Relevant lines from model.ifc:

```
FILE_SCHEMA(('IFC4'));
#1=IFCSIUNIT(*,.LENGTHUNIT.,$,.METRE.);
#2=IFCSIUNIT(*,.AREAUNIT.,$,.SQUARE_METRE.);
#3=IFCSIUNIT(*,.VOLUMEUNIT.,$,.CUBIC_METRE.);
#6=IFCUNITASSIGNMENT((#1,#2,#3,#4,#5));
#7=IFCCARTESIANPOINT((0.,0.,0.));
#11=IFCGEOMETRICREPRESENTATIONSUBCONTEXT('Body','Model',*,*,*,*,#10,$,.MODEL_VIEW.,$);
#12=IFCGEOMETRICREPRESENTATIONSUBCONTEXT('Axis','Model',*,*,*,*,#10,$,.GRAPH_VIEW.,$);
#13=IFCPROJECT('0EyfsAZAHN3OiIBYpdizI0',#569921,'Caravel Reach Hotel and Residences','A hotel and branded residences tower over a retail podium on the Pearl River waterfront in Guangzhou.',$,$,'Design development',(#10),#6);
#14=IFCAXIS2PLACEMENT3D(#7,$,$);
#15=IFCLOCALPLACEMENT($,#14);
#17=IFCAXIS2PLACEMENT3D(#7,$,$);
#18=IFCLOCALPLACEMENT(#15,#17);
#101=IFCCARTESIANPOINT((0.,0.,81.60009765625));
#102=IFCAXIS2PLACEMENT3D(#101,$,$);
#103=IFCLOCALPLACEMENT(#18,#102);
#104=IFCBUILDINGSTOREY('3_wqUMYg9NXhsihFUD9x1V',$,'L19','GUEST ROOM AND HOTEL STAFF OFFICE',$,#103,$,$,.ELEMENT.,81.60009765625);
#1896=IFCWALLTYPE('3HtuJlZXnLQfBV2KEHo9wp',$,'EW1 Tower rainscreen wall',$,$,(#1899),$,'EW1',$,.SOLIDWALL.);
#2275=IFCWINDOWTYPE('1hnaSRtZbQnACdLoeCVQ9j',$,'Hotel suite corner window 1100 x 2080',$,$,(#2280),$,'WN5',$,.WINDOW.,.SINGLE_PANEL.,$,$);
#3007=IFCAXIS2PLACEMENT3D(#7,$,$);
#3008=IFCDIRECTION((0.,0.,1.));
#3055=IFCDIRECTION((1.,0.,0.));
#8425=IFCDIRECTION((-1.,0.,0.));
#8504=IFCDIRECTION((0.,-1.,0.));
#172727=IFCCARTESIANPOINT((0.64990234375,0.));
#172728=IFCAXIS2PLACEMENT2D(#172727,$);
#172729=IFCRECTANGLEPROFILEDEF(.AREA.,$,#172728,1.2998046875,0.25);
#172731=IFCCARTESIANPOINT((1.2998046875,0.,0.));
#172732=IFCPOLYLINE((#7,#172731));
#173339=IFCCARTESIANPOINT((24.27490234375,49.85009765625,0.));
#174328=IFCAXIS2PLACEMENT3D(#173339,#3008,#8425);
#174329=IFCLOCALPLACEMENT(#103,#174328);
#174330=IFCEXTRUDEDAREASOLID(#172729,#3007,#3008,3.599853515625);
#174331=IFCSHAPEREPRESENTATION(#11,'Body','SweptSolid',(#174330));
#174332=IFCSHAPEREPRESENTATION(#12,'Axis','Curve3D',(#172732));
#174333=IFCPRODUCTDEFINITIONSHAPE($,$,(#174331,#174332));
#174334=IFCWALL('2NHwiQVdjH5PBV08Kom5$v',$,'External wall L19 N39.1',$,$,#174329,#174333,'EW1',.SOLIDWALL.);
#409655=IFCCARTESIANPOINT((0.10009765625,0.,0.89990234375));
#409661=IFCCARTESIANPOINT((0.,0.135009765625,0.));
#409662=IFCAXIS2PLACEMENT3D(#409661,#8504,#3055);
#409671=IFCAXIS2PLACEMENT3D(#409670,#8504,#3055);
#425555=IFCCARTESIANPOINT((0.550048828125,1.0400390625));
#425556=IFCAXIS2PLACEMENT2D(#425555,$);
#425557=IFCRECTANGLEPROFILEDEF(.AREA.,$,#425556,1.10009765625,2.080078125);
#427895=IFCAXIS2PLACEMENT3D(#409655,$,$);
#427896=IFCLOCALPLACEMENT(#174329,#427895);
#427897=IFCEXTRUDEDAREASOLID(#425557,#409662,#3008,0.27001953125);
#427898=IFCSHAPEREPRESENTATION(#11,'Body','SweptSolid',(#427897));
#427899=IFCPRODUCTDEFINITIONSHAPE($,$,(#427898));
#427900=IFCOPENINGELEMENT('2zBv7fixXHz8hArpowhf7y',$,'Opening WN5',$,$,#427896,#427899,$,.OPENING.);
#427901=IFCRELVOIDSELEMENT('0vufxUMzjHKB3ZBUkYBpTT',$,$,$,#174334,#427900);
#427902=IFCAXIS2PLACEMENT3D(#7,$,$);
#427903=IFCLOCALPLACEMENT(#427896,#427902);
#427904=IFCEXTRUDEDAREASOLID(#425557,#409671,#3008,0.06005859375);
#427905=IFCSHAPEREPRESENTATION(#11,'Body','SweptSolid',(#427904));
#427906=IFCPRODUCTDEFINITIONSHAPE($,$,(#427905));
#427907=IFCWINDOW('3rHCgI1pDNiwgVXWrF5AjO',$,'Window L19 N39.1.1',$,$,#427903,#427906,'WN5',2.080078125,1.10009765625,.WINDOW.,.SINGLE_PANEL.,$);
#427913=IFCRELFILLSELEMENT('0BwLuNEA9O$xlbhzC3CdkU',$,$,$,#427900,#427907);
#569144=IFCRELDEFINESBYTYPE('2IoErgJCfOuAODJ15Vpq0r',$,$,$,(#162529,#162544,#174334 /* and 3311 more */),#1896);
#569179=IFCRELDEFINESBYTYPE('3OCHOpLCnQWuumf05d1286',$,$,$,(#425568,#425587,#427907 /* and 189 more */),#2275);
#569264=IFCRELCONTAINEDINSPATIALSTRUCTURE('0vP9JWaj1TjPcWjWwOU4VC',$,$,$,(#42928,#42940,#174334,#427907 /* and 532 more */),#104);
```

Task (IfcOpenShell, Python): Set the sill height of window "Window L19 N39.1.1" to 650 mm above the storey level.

```python
import numpy as np
import ifcopenshell
import ifcopenshell.api.geometry
import ifcopenshell.geom
import ifcopenshell.util.element
import ifcopenshell.util.placement
import ifcopenshell.util.shape
import ifcopenshell.util.unit

model = ifcopenshell.open("model.ifc")
unit_scale = ifcopenshell.util.unit.calculate_unit_scale(model)

window = model.by_guid("3rHCgI1pDNiwgVXWrF5AjO")
opening = window.FillsVoids[0].RelatingOpeningElement
storey = ifcopenshell.util.element.get_container(window, ifc_class="IfcBuildingStorey")
level = ifcopenshell.util.placement.get_local_placement(storey.ObjectPlacement)[2, 3]

# The opening's origin need not be at the sill, so measure its lowest point.
shape = ifcopenshell.geom.create_shape(ifcopenshell.geom.settings(), opening)
bottom = ifcopenshell.util.shape.get_shape_bottom_elevation(shape, shape.geometry) / unit_scale
dz = level + 0.65 / unit_scale - bottom

shift = np.array([0.0, 0.0, dz])
# The window is placed relative to its opening, so it follows when the opening moves.
matrix = ifcopenshell.util.placement.get_local_placement(opening.ObjectPlacement)
matrix[:3, 3] += shift
ifcopenshell.api.geometry.edit_object_placement(
    model, product=opening, matrix=matrix, is_si=False, should_transform_children=True
)

print(f"moved by {dz * unit_scale:+.3f} m")

model.write("model_v2.ifc")
```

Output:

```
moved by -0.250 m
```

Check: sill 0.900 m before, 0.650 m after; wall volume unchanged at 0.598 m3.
